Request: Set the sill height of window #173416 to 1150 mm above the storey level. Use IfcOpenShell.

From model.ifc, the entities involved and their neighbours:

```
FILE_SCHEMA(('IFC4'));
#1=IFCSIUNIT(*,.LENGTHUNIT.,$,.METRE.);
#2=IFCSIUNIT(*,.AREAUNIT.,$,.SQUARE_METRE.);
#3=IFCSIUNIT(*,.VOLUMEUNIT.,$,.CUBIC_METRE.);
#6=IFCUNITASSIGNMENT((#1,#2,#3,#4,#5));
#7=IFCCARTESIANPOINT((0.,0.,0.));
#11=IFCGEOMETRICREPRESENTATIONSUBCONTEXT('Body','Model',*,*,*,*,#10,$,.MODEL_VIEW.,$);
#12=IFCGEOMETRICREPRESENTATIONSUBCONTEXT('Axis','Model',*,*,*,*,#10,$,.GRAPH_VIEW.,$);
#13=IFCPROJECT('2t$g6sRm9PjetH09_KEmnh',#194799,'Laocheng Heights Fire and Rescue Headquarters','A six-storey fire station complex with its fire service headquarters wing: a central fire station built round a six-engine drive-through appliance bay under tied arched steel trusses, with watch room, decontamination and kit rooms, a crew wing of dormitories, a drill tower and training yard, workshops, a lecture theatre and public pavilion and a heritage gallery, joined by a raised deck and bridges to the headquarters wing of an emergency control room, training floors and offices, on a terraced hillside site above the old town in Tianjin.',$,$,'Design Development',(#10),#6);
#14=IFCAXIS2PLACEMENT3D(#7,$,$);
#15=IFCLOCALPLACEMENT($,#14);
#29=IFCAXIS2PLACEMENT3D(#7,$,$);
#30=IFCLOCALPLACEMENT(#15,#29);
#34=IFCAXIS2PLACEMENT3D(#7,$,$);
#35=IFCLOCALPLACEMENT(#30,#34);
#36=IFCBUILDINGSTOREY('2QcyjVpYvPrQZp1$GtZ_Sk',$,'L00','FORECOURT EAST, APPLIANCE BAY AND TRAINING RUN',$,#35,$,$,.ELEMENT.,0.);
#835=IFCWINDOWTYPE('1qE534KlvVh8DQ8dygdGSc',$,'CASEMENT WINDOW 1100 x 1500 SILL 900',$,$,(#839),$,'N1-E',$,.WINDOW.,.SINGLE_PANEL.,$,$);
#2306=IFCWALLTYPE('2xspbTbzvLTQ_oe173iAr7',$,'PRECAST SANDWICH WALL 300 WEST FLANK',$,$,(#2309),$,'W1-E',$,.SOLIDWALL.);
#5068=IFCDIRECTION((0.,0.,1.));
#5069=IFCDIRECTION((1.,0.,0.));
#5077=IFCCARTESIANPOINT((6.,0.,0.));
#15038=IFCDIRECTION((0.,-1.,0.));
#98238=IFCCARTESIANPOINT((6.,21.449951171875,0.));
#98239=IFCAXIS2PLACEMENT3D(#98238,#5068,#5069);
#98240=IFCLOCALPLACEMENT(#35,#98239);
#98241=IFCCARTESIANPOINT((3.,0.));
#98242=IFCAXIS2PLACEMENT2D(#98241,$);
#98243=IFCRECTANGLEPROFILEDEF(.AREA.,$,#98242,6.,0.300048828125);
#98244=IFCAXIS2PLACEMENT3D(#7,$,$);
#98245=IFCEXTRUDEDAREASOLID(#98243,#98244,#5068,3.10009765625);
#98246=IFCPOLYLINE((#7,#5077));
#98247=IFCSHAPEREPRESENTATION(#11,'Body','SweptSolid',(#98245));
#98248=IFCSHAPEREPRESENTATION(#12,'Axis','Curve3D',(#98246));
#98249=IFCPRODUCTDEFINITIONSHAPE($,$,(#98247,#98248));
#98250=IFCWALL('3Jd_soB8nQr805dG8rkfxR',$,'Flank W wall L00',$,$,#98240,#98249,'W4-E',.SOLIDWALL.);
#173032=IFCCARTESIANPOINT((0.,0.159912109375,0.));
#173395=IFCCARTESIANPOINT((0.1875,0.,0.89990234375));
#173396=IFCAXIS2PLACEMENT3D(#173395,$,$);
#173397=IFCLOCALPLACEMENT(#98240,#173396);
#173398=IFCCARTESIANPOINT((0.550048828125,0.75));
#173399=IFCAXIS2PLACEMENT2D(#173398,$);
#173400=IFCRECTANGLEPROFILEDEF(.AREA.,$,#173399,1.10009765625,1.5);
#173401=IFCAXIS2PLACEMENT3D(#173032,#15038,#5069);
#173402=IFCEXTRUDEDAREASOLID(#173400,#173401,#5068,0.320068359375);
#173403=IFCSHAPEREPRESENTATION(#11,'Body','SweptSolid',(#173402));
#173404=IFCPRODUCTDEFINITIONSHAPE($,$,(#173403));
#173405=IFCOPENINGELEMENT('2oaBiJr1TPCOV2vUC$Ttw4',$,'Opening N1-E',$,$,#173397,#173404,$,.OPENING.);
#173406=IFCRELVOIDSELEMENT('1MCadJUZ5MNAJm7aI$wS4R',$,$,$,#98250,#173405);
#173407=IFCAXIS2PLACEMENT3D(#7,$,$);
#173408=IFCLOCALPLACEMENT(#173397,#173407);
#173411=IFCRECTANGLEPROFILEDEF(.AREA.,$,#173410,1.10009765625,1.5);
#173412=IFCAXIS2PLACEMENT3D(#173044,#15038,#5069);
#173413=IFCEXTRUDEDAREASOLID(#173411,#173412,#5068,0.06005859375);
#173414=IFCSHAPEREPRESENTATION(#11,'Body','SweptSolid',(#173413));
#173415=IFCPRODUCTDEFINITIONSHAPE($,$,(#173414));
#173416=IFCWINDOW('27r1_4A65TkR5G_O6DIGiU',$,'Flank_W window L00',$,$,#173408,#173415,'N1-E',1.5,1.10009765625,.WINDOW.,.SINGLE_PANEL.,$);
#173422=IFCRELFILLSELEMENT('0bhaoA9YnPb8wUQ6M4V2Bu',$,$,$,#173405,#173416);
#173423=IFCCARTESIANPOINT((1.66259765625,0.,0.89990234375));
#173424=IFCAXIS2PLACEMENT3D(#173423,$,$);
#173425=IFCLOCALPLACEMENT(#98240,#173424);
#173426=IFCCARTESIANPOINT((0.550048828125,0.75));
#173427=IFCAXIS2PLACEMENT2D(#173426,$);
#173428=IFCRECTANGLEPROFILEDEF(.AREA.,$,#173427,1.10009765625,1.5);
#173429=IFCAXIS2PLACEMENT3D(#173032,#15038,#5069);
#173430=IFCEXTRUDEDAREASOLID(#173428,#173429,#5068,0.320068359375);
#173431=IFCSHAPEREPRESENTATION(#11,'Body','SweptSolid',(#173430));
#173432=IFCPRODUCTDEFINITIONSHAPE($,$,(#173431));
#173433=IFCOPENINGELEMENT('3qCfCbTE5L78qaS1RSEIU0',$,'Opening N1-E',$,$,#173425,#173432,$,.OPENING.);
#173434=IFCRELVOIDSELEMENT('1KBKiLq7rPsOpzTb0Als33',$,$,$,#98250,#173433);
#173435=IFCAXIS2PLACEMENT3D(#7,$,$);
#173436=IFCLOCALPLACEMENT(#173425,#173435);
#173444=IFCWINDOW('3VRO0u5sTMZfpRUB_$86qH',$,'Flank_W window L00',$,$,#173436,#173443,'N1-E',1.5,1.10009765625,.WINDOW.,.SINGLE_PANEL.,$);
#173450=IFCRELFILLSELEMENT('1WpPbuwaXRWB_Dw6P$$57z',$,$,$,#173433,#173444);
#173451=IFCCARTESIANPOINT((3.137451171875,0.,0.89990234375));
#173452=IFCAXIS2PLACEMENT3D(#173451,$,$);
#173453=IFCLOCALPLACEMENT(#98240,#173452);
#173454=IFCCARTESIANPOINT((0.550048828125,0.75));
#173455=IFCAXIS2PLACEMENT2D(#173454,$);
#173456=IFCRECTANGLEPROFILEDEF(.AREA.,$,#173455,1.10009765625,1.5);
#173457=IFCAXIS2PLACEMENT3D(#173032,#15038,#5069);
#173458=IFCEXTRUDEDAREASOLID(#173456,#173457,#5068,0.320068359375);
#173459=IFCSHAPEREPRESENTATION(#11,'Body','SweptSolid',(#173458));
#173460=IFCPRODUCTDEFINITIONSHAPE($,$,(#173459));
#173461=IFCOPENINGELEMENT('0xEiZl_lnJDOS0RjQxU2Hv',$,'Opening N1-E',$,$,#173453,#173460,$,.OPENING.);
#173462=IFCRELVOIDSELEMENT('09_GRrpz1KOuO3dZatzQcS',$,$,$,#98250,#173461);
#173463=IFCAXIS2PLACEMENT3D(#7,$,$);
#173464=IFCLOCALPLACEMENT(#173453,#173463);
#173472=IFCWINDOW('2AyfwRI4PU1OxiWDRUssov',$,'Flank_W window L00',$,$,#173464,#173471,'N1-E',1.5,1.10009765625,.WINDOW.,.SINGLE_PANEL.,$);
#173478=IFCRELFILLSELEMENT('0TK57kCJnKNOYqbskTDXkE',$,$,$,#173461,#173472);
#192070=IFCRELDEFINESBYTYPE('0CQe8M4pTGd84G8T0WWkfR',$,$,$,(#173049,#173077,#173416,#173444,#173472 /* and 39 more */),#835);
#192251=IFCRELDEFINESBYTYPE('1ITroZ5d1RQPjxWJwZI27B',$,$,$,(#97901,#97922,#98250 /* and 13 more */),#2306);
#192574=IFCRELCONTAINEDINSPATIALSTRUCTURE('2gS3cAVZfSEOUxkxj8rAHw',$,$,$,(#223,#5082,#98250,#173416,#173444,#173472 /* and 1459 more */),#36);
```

```python
import numpy as np
import ifcopenshell
import ifcopenshell.api.geometry
import ifcopenshell.geom
import ifcopenshell.util.element
import ifcopenshell.util.placement
import ifcopenshell.util.shape
import ifcopenshell.util.unit

model = ifcopenshell.open("model.ifc")
unit_scale = ifcopenshell.util.unit.calculate_unit_scale(model)

window = model.by_guid("27r1_4A65TkR5G_O6DIGiU")
opening = window.FillsVoids[0].RelatingOpeningElement
storey = ifcopenshell.util.element.get_container(window, ifc_class="IfcBuildingStorey")
level = ifcopenshell.util.placement.get_local_placement(storey.ObjectPlacement)[2, 3]

# The opening's origin need not be at the sill, so measure its lowest point.
shape = ifcopenshell.geom.create_shape(ifcopenshell.geom.settings(), opening)
bottom = ifcopenshell.util.shape.get_shape_bottom_elevation(shape, shape.geometry) / unit_scale
dz = level + 1.15 / unit_scale - bottom

shift = np.array([0.0, 0.0, dz])
# The window is placed relative to its opening, so it follows when the opening moves.
matrix = ifcopenshell.util.placement.get_local_placement(opening.ObjectPlacement)
matrix[:3, 3] += shift
ifcopenshell.api.geometry.edit_object_placement(
    model, product=opening, matrix=matrix, is_si=False, should_transform_children=True
)

print(f"moved by {dz * unit_scale:+.3f} m")

model.write("model_updated.ifc")
```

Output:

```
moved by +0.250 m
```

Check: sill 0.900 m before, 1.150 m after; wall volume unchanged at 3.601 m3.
